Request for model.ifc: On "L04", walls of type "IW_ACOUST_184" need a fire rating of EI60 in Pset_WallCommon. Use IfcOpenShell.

First a look at what the model holds.

```python
import ifcopenshell
import ifcopenshell.util.element

model = ifcopenshell.open("model.ifc")
print(model.schema)
storey = next(s for s in model.by_type("IfcBuildingStorey") if s.Name == "L04")
walls = [e for e in ifcopenshell.util.element.get_decomposition(storey) if e.is_a("IfcWall")]
seen = {}
for e in walls:
    element_type = ifcopenshell.util.element.get_type(e)
    key = (element_type.Name if element_type != e and element_type else None, ifcopenshell.util.element.get_pset(e, "Pset_WallCommon", "FireRating"))
    seen[key] = seen.get(key, 0) + 1
for (name, value), count in sorted(seen.items(), key=str):
    print(count, "x", name, "|", value)
```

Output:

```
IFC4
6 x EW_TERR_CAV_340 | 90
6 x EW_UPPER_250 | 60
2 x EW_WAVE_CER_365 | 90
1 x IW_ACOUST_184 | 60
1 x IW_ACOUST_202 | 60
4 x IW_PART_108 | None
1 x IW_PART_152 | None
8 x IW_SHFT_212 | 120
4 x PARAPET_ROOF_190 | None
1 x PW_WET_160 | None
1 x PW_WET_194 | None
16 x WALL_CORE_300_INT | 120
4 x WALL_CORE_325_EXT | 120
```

```python
import ifcopenshell
import ifcopenshell.api.pset
import ifcopenshell.util.element

model = ifcopenshell.open("model.ifc")

storey = next(s for s in model.by_type("IfcBuildingStorey") if s.Name == "L04")
walls = [e for e in ifcopenshell.util.element.get_decomposition(storey) if e.is_a("IfcWall")]

count = 0
for e in walls:
    element_type = ifcopenshell.util.element.get_type(e)
    if element_type in (None, e) or element_type.Name != "IW_ACOUST_184":
        continue
    # add_pset returns the element's existing set when there is one.
    pset = ifcopenshell.api.pset.add_pset(model, product=e, name="Pset_WallCommon")
    ifcopenshell.api.pset.edit_pset(model, pset=pset, properties={"FireRating": "EI60"})
    count += 1

print(count, "walls updated")

model.write("model-out.ifc")
```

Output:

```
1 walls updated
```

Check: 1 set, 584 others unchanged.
